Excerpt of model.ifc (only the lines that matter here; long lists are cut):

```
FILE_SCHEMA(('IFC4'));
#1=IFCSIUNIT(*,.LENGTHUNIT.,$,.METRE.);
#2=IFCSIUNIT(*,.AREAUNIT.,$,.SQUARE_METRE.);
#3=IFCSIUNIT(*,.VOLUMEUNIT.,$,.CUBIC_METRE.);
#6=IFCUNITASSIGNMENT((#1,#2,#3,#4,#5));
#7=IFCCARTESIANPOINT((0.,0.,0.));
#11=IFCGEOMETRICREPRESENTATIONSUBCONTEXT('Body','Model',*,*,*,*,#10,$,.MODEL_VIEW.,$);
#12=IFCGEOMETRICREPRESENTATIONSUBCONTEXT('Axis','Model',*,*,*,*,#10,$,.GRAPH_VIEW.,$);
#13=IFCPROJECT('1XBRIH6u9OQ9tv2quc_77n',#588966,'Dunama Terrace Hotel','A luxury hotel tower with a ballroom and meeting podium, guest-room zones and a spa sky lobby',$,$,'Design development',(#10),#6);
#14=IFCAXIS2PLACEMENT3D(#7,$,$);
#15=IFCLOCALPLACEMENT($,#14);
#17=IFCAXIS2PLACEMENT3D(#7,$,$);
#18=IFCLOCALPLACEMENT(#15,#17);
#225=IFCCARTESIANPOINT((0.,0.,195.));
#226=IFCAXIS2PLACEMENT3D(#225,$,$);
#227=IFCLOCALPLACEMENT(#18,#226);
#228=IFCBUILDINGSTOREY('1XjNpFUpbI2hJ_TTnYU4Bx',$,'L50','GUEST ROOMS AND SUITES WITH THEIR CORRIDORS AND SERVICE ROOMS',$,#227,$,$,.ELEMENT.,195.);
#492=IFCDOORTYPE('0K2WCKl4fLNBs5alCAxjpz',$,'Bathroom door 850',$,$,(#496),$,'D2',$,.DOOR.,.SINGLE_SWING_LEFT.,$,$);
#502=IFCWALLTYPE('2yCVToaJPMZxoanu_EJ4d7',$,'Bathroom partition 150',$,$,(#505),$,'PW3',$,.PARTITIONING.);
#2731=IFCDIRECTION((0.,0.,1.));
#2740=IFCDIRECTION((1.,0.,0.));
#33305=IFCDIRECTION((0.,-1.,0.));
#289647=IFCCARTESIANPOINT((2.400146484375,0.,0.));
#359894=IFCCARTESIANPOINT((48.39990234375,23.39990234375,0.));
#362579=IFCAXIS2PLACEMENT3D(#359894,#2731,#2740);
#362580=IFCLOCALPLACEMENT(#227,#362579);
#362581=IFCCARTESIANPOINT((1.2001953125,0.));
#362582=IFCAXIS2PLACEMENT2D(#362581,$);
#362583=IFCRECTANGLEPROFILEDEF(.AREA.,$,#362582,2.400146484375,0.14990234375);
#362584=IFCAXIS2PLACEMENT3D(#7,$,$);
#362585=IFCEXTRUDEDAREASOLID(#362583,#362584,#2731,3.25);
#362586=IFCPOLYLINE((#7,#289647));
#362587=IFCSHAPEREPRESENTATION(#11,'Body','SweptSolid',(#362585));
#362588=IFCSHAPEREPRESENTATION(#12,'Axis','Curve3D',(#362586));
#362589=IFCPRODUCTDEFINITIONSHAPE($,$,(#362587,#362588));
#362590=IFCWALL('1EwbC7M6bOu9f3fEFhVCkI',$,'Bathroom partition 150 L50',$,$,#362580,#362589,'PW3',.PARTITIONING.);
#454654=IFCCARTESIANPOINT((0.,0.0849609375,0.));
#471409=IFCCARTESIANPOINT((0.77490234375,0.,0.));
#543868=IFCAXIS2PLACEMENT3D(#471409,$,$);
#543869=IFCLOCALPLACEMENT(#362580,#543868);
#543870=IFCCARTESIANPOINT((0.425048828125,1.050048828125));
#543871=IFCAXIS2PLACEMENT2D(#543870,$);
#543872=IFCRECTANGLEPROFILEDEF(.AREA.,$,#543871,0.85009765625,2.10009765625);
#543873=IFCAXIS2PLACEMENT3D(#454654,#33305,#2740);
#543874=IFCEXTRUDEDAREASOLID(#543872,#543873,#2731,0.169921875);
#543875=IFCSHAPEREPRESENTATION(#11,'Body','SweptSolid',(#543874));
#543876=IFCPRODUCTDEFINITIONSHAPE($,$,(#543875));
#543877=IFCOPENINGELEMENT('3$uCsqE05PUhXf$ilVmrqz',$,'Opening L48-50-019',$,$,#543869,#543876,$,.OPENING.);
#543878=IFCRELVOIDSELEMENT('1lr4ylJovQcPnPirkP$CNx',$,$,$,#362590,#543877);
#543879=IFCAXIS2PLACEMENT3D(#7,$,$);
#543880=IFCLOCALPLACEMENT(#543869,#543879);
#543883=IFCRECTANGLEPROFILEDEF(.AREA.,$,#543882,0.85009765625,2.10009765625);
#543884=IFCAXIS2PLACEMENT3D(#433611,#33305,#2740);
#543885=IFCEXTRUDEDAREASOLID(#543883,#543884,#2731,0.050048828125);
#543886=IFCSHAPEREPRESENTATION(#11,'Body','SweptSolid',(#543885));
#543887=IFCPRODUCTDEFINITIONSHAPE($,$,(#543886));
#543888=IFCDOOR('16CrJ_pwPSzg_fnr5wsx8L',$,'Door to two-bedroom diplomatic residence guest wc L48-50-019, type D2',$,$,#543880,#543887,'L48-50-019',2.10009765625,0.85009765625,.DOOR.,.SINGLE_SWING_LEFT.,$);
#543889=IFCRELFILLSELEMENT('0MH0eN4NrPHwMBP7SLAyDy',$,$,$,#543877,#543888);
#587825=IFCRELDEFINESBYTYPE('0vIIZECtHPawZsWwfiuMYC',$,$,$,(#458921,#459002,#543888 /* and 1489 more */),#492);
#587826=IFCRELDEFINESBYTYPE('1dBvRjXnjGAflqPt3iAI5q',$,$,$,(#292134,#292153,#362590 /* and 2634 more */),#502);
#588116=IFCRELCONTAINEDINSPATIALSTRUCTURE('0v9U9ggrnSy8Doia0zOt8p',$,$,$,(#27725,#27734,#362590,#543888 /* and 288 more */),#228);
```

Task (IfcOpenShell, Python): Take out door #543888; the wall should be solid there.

```python
import ifcopenshell
import ifcopenshell.api.feature
import ifcopenshell.api.root
import ifcopenshell.geom
import ifcopenshell.util.shape

model = ifcopenshell.open("model.ifc")
settings = ifcopenshell.geom.settings()


def volume(element):
    """Net volume in cubic metres, openings subtracted."""
    shape = ifcopenshell.geom.create_shape(settings, element)
    return ifcopenshell.util.shape.get_volume(shape.geometry)


door = model.by_id(543888)
opening = door.FillsVoids[0].RelatingOpeningElement
wall = opening.VoidsElements[0].RelatingBuildingElement
before = volume(wall)

ifcopenshell.api.root.remove_product(model, product=door)
ifcopenshell.api.feature.remove_feature(model, feature=opening)

after = volume(wall)

print(f"wall volume {before:.3f} -> {after:.3f} m3")

model.write("model_rev.ifc")
```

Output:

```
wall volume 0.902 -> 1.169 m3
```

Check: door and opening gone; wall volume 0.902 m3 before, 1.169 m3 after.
